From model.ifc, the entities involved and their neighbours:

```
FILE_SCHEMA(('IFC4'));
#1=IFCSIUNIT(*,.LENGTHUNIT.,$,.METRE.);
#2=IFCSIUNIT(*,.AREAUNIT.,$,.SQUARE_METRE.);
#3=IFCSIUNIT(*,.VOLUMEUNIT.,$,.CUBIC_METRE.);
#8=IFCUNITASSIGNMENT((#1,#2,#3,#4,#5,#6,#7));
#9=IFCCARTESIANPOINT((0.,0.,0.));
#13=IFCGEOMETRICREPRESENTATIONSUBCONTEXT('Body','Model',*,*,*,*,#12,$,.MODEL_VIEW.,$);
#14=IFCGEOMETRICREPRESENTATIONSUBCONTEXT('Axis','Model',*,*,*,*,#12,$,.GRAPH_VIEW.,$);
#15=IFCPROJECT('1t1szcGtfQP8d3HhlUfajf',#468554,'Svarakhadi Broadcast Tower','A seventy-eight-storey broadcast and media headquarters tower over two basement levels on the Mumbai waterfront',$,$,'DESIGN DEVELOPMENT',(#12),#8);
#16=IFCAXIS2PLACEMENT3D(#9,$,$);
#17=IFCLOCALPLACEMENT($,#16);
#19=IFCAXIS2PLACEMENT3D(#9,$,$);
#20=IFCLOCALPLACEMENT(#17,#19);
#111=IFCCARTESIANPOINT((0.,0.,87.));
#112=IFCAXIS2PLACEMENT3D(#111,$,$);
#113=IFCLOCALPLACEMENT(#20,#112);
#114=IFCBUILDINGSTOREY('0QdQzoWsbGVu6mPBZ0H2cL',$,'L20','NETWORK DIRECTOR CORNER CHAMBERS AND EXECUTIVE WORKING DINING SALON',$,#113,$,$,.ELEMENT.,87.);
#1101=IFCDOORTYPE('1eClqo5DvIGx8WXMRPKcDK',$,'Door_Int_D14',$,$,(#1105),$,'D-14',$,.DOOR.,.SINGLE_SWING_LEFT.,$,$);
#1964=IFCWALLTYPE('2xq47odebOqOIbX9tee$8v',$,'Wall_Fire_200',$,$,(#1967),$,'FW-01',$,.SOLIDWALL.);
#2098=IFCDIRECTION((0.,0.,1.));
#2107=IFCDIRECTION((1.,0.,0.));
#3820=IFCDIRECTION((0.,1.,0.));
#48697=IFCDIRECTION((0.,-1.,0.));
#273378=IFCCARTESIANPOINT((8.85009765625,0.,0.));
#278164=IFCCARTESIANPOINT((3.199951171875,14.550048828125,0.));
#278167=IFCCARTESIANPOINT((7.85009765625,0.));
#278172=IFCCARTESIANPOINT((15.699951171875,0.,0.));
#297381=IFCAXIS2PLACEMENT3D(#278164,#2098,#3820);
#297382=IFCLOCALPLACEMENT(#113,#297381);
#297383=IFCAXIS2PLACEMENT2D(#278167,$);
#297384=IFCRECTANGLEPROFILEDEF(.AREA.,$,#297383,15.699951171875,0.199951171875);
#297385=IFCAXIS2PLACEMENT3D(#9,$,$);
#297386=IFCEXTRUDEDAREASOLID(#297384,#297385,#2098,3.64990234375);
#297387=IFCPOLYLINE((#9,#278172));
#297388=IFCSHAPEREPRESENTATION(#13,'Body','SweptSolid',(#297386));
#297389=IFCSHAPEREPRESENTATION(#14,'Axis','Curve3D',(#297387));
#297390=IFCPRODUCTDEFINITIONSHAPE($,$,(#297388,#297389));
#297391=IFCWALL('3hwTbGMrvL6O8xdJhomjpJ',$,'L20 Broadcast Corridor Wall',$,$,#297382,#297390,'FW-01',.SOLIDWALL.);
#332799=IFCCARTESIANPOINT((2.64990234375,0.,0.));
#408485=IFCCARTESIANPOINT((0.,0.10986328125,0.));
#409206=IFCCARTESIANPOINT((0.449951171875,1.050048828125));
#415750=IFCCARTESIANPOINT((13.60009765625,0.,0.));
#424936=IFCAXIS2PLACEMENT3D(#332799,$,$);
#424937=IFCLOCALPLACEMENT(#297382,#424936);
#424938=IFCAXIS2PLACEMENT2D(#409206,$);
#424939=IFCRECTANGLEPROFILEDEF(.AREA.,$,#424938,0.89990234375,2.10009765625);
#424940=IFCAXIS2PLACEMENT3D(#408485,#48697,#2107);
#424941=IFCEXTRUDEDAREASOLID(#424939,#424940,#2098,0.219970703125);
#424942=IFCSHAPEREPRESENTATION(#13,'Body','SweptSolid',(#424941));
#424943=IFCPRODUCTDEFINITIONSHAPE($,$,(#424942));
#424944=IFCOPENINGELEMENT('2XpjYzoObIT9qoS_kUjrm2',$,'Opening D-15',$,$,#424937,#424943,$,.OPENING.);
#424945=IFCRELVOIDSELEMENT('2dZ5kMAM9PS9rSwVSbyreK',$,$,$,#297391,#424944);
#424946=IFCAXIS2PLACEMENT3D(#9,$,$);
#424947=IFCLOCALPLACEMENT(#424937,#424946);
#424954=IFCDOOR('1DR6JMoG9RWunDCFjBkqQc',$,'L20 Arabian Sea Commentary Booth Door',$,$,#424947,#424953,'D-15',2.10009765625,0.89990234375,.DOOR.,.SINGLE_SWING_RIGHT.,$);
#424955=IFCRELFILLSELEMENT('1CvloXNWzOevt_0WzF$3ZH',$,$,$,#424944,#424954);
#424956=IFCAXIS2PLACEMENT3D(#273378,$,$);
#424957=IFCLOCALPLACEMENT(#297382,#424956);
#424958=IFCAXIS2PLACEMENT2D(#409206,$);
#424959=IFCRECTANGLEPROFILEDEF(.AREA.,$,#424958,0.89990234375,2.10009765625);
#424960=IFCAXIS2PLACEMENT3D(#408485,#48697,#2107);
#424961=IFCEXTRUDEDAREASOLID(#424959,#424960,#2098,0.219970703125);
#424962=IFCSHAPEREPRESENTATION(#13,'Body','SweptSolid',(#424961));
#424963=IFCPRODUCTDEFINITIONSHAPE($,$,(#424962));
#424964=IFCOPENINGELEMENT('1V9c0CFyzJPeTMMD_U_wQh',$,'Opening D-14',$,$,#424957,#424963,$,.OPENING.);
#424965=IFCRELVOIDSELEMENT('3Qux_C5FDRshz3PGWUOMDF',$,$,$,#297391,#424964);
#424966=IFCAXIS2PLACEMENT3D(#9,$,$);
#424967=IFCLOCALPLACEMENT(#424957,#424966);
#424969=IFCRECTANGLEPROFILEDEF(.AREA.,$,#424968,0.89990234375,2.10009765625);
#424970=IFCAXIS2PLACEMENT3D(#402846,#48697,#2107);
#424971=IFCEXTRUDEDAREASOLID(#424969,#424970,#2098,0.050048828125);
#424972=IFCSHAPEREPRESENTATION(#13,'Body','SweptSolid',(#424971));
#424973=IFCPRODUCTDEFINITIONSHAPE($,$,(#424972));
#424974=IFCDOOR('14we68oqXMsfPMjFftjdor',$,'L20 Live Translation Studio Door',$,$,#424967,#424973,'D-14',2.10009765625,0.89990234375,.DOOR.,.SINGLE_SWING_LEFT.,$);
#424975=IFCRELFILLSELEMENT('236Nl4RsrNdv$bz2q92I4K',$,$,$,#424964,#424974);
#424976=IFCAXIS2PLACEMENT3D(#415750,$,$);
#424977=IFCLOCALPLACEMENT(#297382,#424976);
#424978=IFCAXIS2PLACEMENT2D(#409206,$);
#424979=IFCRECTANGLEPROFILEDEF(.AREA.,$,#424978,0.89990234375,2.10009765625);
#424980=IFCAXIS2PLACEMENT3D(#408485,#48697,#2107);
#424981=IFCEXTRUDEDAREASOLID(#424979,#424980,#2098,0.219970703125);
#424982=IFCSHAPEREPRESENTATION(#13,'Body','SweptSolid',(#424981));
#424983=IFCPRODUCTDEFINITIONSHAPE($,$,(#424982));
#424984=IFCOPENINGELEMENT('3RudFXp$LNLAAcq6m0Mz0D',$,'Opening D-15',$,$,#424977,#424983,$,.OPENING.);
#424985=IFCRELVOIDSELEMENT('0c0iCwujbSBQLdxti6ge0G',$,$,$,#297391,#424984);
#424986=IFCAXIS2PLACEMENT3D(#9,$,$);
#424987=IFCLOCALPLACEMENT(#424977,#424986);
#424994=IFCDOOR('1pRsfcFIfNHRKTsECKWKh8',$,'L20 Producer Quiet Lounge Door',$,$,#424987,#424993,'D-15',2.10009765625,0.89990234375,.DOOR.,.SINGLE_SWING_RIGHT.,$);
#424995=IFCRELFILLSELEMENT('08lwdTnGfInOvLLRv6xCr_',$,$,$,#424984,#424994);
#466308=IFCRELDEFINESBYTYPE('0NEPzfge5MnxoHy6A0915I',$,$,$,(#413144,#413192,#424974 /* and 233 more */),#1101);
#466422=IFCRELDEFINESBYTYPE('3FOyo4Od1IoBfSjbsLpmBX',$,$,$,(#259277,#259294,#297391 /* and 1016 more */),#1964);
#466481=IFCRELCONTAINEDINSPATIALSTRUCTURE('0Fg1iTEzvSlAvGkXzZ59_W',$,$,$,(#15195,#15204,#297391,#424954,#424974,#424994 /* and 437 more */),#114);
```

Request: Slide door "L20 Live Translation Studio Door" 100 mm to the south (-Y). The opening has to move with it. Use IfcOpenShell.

```python
import ifcopenshell
import ifcopenshell.api.geometry
import ifcopenshell.util.placement
import ifcopenshell.util.unit

model = ifcopenshell.open("model.ifc")
unit_scale = ifcopenshell.util.unit.calculate_unit_scale(model)

door = model.by_guid("14we68oqXMsfPMjFftjdor")
opening = door.FillsVoids[0].RelatingOpeningElement
wall = opening.VoidsElements[0].RelatingBuildingElement

wall_matrix = ifcopenshell.util.placement.get_local_placement(wall.ObjectPlacement)
shift = wall_matrix[:3, 0] * -0.1 / unit_scale
before = ifcopenshell.util.placement.get_local_placement(door.ObjectPlacement)[:3, 3].copy()

# The door is placed relative to its opening, so it follows when the opening moves.
matrix = ifcopenshell.util.placement.get_local_placement(opening.ObjectPlacement)
matrix[:3, 3] += shift
ifcopenshell.api.geometry.edit_object_placement(
    model, product=opening, matrix=matrix, is_si=False, should_transform_children=True
)

after = ifcopenshell.util.placement.get_local_placement(door.ObjectPlacement)[:3, 3]
print("door moved by", (after - before).round(3) + 0.0)

model.write("model_edited.ifc")
```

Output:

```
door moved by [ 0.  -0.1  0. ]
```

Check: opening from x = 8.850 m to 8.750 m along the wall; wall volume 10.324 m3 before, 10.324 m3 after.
